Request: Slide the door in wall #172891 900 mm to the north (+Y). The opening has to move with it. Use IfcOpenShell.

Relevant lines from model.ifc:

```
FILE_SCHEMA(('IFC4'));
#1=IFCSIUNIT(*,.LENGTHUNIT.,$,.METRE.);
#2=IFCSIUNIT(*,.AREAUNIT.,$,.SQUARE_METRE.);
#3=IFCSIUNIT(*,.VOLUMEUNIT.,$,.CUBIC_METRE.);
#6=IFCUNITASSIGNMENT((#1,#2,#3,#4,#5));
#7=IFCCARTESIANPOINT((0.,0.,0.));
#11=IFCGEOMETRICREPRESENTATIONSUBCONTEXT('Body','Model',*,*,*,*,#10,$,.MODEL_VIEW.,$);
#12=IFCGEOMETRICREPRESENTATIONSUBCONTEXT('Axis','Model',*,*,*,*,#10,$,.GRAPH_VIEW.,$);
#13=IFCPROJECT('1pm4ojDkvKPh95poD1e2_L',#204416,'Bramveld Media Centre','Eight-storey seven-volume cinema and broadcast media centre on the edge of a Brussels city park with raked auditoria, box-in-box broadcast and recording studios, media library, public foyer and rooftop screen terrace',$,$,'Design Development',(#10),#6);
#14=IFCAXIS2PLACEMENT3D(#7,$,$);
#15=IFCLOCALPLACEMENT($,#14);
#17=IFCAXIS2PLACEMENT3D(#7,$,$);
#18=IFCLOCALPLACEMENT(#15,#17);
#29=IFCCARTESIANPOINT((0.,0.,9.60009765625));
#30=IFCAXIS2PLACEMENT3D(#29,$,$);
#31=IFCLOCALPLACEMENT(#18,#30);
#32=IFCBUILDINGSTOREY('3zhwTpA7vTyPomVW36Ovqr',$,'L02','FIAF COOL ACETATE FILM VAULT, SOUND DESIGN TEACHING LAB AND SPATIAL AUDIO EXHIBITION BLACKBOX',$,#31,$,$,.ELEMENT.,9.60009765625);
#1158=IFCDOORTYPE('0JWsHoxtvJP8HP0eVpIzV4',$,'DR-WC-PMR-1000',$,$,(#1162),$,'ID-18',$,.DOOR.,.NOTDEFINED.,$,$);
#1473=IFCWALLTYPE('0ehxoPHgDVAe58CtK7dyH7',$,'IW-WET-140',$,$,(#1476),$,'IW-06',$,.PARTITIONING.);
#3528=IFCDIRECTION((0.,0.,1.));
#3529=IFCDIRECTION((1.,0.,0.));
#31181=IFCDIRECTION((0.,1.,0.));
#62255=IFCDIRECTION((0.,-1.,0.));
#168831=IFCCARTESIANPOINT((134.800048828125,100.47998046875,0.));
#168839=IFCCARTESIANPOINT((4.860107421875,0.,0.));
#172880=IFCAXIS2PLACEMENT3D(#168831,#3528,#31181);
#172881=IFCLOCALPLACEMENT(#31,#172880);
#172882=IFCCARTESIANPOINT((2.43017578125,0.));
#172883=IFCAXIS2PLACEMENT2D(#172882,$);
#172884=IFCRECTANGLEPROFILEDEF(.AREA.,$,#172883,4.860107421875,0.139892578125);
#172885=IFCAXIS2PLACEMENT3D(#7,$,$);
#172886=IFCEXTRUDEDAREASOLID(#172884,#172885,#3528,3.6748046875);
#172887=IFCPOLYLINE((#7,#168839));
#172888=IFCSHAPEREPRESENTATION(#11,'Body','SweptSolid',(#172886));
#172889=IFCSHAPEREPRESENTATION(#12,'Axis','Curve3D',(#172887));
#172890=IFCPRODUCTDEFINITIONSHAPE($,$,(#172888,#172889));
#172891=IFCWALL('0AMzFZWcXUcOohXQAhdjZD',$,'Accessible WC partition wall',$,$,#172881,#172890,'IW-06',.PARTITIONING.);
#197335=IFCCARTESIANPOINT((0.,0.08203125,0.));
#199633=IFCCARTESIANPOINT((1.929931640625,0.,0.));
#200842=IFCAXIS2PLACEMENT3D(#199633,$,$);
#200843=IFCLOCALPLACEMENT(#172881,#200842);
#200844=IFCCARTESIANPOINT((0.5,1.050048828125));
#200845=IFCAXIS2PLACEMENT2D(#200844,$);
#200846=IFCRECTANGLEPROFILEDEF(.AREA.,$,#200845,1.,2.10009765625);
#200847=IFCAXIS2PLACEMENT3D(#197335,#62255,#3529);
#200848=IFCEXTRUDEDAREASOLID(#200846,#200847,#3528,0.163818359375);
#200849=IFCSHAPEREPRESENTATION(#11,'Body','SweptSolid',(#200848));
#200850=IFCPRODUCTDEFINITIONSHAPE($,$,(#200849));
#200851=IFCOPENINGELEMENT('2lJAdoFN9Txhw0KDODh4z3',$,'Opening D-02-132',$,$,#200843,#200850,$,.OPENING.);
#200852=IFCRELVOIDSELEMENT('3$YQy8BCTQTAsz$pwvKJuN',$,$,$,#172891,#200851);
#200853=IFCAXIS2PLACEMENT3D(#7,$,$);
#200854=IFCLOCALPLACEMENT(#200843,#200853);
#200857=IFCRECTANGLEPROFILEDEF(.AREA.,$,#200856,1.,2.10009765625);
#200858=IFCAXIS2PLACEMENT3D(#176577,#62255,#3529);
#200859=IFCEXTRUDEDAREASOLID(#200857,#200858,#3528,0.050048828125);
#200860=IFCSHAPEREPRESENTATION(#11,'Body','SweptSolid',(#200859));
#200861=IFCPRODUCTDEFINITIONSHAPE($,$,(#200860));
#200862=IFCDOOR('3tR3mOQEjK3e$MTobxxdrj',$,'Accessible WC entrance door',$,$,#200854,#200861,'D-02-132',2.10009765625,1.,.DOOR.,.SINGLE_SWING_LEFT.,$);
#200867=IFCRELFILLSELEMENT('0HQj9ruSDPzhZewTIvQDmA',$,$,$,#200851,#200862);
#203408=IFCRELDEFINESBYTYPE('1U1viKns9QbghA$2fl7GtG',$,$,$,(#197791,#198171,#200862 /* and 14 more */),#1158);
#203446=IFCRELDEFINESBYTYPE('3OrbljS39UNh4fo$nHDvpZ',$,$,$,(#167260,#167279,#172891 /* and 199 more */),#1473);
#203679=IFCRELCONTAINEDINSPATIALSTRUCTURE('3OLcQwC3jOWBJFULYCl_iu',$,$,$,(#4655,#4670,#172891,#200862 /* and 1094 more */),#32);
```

```python
import ifcopenshell
import ifcopenshell.api.geometry
import ifcopenshell.util.placement

model = ifcopenshell.open("model.ifc")

door = model.by_guid("3tR3mOQEjK3e$MTobxxdrj")
opening = door.FillsVoids[0].RelatingOpeningElement
wall = opening.VoidsElements[0].RelatingBuildingElement

wall_matrix = ifcopenshell.util.placement.get_local_placement(wall.ObjectPlacement)
shift = wall_matrix[:3, 0] * 0.9
before = ifcopenshell.util.placement.get_local_placement(door.ObjectPlacement)[:3, 3].copy()

# The door is placed relative to its opening, so it follows when the opening moves.
matrix = ifcopenshell.util.placement.get_local_placement(opening.ObjectPlacement)
matrix[:3, 3] += shift
ifcopenshell.api.geometry.edit_object_placement(
    model, product=opening, matrix=matrix, is_si=False, should_transform_children=True
)

after = ifcopenshell.util.placement.get_local_placement(door.ObjectPlacement)[:3, 3]
print("door moved by", (after - before).round(3) + 0.0)

model.write("model_edited.ifc")
```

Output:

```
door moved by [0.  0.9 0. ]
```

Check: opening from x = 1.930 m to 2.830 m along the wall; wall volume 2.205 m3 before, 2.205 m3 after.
